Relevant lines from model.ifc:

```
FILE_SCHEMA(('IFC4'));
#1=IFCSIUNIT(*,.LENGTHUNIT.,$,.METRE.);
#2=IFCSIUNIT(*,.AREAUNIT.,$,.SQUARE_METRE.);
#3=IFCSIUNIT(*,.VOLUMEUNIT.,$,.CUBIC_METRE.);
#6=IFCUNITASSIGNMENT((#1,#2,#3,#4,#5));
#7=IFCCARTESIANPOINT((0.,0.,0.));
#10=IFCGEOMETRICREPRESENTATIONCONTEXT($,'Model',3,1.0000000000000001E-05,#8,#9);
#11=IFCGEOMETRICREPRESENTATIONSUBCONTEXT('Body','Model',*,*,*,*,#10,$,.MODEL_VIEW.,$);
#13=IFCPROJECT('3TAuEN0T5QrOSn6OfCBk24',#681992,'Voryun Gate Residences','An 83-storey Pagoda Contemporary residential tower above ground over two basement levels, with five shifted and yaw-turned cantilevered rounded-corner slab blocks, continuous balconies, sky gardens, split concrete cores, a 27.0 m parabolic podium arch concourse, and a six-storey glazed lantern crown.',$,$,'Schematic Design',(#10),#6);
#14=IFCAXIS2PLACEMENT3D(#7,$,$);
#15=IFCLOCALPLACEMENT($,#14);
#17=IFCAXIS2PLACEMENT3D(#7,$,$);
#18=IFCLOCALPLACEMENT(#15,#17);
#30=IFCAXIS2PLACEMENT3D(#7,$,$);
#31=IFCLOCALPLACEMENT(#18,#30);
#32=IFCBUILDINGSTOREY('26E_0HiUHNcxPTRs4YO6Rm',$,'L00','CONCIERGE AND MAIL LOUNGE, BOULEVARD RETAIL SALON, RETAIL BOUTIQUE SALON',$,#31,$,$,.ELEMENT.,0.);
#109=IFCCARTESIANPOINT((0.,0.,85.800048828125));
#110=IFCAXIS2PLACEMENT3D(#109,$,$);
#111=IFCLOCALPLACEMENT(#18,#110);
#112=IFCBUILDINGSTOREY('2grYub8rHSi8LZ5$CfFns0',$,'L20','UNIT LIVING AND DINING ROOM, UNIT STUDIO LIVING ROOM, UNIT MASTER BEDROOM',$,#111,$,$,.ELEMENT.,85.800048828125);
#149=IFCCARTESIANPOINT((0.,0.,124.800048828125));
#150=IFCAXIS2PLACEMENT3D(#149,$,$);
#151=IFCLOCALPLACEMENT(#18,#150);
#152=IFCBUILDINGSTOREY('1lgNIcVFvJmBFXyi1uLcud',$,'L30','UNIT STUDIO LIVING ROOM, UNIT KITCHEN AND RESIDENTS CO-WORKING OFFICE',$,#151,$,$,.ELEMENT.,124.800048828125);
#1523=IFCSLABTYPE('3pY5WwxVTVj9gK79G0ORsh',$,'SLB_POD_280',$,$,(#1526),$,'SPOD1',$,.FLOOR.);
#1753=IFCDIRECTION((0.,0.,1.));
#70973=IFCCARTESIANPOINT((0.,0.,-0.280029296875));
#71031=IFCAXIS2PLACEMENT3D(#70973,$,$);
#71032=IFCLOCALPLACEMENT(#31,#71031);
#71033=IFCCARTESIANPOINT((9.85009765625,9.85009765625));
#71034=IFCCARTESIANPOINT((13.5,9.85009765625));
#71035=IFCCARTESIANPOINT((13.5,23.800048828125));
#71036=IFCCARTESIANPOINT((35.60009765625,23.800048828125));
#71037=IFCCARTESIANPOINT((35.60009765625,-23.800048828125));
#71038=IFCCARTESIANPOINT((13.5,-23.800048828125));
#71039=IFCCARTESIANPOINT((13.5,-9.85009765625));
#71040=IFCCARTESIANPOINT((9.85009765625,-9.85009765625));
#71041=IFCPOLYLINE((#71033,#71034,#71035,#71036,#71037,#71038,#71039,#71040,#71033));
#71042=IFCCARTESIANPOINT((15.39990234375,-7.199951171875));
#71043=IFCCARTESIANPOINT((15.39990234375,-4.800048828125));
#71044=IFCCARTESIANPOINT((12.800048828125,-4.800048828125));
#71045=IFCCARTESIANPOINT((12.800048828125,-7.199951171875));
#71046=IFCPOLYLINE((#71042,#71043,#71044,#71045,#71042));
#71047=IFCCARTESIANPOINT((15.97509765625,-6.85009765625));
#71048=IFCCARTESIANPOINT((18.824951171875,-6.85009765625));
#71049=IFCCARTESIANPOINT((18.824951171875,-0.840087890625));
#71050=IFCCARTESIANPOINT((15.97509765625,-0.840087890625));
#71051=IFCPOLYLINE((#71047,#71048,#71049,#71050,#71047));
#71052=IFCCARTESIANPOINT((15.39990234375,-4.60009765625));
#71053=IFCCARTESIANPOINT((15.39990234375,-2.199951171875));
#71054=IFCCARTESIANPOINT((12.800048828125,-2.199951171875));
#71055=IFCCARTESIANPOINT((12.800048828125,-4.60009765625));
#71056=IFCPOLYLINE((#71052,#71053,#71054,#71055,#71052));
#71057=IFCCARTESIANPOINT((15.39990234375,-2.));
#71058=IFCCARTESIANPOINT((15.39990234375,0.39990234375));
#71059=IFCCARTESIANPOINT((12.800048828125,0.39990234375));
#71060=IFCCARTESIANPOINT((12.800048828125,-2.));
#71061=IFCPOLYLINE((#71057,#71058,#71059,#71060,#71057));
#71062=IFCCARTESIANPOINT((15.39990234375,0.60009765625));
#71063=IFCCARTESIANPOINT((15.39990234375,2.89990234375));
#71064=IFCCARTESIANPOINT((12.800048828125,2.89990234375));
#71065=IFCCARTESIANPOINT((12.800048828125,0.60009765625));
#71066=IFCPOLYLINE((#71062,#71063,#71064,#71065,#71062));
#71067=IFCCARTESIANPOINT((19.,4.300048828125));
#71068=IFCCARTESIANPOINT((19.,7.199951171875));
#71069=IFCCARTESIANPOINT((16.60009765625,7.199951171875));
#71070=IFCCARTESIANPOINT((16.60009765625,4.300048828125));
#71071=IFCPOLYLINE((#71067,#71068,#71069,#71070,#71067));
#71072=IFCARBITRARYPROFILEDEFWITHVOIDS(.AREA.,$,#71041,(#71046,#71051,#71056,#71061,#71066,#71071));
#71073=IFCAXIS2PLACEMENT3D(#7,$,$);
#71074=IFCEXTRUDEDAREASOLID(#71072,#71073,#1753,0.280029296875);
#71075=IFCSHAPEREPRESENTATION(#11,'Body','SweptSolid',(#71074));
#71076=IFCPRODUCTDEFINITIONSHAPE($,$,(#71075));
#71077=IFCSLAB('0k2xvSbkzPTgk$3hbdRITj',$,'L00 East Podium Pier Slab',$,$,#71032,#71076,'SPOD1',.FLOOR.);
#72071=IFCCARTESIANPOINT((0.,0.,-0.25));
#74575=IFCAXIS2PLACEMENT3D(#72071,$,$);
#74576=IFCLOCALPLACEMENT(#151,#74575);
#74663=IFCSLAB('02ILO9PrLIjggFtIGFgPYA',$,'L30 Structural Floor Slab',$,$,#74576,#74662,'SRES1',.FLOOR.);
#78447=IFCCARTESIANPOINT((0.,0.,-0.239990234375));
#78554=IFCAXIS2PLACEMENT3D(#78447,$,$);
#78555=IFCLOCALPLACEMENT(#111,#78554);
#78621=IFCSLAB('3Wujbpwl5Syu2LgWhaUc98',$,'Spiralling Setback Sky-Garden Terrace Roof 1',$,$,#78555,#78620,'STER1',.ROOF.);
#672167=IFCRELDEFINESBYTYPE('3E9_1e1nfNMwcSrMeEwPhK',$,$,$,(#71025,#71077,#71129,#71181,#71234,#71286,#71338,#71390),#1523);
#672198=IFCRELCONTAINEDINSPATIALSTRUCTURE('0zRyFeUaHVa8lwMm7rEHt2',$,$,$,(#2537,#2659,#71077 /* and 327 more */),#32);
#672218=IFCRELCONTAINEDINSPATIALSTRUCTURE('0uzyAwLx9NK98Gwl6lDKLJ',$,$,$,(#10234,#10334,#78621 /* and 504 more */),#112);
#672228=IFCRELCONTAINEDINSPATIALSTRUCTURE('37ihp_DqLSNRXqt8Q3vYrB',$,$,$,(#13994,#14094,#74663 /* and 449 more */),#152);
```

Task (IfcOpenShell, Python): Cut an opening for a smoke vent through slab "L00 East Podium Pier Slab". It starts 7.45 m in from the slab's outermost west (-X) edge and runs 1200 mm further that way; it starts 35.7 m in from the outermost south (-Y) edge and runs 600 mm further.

```python
import numpy as np
import ifcopenshell
import ifcopenshell.api.feature
import ifcopenshell.api.geometry
import ifcopenshell.api.root
import ifcopenshell.geom
import ifcopenshell.util.placement
import ifcopenshell.util.representation
import ifcopenshell.util.shape
import ifcopenshell.util.unit

model = ifcopenshell.open("model.ifc")
unit_scale = ifcopenshell.util.unit.calculate_unit_scale(model)
settings = ifcopenshell.geom.settings()


def volume(element):
    """Net volume in cubic metres, openings subtracted."""
    shape = ifcopenshell.geom.create_shape(settings, element)
    return ifcopenshell.util.shape.get_volume(shape.geometry)


slab = model.by_guid("0k2xvSbkzPTgk$3hbdRITj")
before = volume(slab)

# Extent in the slab's own axes, in metres. The edges named are its -X and -Y sides.
slab_shape = ifcopenshell.geom.create_shape(settings, slab)
vertices = ifcopenshell.util.shape.get_vertices(slab_shape.geometry)
x_min, y_min, bottom = vertices.min(axis=0)
top = vertices[:, 2].max()

opening = ifcopenshell.api.root.create_entity(model, ifc_class="IfcOpeningElement", name="Smoke vent opening", predefined_type="OPENING")
context = ifcopenshell.util.representation.get_context(model, "Model", "Body", "MODEL_VIEW")
width, depth = 1.2, 0.6
outline = [(0.0, 0.0), (width, 0.0), (width, depth), (0.0, depth), (0.0, 0.0)]
# Overshoot both faces by 50 mm so the cut is clean.
shape = ifcopenshell.api.geometry.add_slab_representation(
    model, context=context, depth=top - bottom + 0.1, polyline=outline
)
ifcopenshell.api.geometry.assign_representation(model, product=opening, representation=shape)

matrix = ifcopenshell.util.placement.get_local_placement(slab.ObjectPlacement)
matrix[:, 3] = matrix @ np.append(np.array([x_min + 7.45, y_min + 35.7, bottom - 0.05]) / unit_scale, 1.0)
ifcopenshell.api.geometry.edit_object_placement(model, product=opening, matrix=matrix, is_si=False)
ifcopenshell.api.feature.add_feature(model, feature=opening, element=slab)

after = volume(slab)

print(f"slab volume {before:.3f} -> {after:.3f} m3")

model.write("model-out.ifc")
```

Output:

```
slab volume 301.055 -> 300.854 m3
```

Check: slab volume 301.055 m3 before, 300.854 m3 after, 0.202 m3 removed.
